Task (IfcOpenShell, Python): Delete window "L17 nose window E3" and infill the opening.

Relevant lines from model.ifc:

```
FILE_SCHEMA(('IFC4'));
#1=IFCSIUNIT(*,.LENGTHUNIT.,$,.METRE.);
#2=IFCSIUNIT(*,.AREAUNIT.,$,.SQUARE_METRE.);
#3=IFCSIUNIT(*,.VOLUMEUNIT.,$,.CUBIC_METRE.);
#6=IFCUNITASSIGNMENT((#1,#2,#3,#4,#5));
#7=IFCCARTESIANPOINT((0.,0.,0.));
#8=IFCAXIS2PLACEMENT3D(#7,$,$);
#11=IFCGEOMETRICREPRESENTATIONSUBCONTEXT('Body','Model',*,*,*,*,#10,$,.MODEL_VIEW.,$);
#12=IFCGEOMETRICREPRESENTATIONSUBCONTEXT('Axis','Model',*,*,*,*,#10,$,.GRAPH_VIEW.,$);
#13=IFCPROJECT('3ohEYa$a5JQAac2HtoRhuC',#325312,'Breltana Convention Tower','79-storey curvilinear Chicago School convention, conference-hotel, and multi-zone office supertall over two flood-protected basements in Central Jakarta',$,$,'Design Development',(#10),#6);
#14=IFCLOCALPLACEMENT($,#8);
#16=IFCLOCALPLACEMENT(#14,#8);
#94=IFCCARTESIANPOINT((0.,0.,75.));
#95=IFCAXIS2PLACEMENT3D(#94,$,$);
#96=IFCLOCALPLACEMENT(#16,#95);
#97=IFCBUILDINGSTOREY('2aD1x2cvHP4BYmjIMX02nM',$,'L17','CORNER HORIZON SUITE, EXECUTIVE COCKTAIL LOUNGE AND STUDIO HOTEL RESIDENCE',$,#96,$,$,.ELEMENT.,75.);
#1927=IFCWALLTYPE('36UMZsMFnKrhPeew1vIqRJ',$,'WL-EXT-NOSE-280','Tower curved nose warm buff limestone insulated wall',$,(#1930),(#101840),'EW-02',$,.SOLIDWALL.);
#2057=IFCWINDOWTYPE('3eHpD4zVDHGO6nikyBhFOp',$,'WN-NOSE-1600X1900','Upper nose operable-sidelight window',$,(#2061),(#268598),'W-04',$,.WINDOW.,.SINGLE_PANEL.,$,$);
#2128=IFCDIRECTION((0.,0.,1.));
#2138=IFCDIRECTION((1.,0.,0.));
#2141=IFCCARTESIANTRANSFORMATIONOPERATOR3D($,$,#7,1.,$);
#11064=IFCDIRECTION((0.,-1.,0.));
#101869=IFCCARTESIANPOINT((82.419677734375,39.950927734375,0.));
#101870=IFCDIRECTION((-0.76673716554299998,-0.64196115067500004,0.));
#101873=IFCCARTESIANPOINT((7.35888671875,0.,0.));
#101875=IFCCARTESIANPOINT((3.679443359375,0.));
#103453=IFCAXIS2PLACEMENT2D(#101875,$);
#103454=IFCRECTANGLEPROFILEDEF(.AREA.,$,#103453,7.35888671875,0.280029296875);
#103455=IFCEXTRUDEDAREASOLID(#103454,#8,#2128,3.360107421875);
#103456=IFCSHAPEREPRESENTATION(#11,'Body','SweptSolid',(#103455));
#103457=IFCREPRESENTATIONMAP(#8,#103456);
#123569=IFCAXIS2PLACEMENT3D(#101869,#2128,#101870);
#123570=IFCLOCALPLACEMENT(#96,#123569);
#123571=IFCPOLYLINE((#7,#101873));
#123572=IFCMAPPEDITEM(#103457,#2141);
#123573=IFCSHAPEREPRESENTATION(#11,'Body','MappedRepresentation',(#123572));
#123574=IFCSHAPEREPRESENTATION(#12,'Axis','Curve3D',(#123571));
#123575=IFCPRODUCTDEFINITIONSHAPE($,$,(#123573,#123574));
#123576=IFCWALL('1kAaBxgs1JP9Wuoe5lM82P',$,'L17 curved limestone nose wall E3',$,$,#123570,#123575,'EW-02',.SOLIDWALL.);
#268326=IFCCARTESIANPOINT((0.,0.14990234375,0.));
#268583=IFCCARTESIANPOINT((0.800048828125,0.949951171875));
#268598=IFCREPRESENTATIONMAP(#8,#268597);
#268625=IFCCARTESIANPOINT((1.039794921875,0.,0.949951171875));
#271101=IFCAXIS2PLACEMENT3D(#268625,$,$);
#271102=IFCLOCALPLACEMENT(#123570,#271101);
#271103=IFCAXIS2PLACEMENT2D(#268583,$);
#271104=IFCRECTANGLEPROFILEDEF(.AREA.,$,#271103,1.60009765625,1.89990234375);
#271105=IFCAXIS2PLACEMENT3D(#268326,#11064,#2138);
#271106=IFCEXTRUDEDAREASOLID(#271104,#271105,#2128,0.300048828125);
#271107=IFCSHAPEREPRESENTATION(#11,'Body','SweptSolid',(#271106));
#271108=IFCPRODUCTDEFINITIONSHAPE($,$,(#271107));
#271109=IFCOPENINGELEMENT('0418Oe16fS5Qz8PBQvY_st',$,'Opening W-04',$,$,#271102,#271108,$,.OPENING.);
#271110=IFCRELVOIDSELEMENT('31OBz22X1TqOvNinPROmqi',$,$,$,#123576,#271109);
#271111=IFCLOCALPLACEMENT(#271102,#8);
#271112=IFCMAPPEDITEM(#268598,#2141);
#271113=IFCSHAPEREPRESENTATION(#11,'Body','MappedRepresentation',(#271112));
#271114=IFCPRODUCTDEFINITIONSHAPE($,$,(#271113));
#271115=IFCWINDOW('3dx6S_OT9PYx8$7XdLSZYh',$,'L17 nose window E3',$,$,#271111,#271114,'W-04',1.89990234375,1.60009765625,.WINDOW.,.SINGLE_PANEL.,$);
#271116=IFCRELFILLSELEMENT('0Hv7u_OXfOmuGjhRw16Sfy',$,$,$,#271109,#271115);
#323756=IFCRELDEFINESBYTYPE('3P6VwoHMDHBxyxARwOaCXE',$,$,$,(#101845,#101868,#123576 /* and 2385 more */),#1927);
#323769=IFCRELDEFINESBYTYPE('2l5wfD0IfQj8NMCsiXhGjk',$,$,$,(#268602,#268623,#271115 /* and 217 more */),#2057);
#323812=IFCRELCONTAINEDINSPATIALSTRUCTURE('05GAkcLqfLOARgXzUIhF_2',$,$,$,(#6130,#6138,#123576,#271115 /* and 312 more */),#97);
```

```python
import ifcopenshell
import ifcopenshell.api.feature
import ifcopenshell.api.root
import ifcopenshell.geom
import ifcopenshell.util.shape

model = ifcopenshell.open("model.ifc")
settings = ifcopenshell.geom.settings()


def volume(element):
    """Net volume in cubic metres, openings subtracted."""
    shape = ifcopenshell.geom.create_shape(settings, element)
    return ifcopenshell.util.shape.get_volume(shape.geometry)


window = model.by_guid("3dx6S_OT9PYx8$7XdLSZYh")
opening = window.FillsVoids[0].RelatingOpeningElement
wall = opening.VoidsElements[0].RelatingBuildingElement
before = volume(wall)

ifcopenshell.api.root.remove_product(model, product=window)
ifcopenshell.api.feature.remove_feature(model, feature=opening)

after = volume(wall)

print(f"wall volume {before:.3f} -> {after:.3f} m3")

model.write("model_v2.ifc")
```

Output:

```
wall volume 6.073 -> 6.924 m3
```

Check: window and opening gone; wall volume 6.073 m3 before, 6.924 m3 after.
